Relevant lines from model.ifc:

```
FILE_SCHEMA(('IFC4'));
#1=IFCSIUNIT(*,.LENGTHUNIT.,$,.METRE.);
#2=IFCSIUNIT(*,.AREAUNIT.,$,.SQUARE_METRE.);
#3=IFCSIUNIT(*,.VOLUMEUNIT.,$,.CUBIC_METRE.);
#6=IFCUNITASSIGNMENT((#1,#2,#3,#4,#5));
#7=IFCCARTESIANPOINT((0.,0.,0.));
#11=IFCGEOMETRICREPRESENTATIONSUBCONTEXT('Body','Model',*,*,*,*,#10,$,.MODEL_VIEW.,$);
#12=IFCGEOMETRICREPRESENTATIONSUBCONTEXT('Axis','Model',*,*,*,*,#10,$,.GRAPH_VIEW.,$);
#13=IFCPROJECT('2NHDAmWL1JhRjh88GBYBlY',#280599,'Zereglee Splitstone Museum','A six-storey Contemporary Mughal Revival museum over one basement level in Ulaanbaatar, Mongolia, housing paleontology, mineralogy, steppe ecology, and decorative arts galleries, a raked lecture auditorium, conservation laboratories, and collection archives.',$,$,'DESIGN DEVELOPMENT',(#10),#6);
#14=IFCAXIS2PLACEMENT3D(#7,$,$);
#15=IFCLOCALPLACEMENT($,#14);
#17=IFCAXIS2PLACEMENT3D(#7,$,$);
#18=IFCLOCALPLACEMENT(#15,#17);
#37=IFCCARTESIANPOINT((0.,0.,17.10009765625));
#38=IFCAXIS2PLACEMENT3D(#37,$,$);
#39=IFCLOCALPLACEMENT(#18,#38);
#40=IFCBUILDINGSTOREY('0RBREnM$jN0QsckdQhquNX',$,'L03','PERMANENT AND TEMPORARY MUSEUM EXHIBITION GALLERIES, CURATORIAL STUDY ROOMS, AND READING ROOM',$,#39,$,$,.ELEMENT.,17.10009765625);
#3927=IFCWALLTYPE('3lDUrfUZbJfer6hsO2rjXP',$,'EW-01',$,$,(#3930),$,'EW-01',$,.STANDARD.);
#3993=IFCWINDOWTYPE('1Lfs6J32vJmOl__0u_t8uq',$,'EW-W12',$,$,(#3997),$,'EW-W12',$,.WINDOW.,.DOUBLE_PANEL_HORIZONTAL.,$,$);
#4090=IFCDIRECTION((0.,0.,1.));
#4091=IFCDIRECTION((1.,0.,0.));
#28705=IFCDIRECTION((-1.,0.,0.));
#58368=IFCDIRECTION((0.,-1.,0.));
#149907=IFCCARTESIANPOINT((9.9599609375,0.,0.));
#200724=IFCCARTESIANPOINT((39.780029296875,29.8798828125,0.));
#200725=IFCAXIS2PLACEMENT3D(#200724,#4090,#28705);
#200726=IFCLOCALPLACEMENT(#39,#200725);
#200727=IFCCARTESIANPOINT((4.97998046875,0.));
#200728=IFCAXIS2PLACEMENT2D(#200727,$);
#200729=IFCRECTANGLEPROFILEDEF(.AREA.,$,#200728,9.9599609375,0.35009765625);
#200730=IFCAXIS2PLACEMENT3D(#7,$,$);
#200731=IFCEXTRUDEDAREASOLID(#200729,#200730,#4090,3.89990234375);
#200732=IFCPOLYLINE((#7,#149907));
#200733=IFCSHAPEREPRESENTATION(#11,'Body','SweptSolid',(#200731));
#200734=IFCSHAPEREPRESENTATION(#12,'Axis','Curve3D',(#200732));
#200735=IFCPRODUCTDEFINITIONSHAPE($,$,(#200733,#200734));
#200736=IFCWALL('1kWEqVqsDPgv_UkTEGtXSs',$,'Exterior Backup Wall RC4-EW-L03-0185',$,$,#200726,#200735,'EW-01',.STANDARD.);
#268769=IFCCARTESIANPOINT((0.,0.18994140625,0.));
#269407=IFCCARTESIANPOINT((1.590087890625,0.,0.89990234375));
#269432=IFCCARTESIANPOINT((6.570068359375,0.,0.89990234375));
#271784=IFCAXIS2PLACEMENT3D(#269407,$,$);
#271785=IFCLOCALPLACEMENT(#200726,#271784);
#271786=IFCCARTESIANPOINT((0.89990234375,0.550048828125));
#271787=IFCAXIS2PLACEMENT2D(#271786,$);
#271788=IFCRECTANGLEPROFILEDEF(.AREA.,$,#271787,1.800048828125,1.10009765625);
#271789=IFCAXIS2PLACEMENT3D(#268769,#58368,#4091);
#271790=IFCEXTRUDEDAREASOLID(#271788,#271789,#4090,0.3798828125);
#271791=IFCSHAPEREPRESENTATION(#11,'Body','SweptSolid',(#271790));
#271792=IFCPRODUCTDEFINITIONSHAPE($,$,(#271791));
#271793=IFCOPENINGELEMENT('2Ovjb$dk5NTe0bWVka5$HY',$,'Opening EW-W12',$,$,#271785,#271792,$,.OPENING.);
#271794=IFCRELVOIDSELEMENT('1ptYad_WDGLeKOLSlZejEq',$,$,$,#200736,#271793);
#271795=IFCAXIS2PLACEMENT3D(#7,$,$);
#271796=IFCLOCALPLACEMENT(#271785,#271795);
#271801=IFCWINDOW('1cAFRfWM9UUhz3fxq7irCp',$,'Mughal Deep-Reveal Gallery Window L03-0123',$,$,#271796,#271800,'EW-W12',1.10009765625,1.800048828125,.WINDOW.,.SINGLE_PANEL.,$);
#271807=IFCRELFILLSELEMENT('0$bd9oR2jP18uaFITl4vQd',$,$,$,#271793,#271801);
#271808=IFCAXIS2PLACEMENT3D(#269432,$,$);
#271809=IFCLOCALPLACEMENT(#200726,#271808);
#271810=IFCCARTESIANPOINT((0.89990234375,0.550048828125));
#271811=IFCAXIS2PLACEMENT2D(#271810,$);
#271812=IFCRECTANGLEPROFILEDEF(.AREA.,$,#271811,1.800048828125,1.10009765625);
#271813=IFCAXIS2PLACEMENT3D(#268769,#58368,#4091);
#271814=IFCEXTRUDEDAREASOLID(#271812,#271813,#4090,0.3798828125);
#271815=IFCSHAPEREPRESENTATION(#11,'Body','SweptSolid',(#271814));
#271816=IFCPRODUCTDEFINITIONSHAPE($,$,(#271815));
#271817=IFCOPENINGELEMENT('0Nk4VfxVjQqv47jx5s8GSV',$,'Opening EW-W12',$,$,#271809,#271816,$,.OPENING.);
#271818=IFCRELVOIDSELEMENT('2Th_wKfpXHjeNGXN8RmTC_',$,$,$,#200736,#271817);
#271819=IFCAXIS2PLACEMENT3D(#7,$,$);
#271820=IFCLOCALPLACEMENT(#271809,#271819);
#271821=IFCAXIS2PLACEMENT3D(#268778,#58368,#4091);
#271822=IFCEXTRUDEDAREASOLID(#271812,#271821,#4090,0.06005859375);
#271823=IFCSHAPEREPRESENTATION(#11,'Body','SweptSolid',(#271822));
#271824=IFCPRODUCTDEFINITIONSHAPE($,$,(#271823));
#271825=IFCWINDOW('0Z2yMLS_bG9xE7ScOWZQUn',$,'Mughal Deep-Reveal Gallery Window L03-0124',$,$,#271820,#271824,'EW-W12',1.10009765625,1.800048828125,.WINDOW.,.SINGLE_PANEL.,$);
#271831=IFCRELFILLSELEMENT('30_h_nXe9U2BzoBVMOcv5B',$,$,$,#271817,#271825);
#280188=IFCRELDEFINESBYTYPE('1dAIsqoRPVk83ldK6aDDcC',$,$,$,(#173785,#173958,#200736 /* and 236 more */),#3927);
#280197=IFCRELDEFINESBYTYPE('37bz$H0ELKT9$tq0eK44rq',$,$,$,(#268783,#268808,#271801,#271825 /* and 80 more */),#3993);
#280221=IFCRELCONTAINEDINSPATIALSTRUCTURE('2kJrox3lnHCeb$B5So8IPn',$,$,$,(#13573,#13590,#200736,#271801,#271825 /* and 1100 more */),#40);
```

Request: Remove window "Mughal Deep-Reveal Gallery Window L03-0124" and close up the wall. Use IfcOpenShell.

```python
import ifcopenshell
import ifcopenshell.api.feature
import ifcopenshell.api.root
import ifcopenshell.geom
import ifcopenshell.util.shape

model = ifcopenshell.open("model.ifc")
settings = ifcopenshell.geom.settings()


def volume(element):
    """Net volume in cubic metres, openings subtracted."""
    shape = ifcopenshell.geom.create_shape(settings, element)
    return ifcopenshell.util.shape.get_volume(shape.geometry)


window = model.by_guid("0Z2yMLS_bG9xE7ScOWZQUn")
opening = window.FillsVoids[0].RelatingOpeningElement
wall = opening.VoidsElements[0].RelatingBuildingElement
before = volume(wall)

ifcopenshell.api.root.remove_product(model, product=window)
ifcopenshell.api.feature.remove_feature(model, feature=opening)

after = volume(wall)

print(f"wall volume {before:.3f} -> {after:.3f} m3")

model.write("model_edited.ifc")
```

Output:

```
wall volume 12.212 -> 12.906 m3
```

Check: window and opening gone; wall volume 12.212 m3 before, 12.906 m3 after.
